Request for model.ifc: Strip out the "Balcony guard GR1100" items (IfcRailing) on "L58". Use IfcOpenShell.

First a look at what the model holds.

```python
import ifcopenshell
import ifcopenshell.util.element

model = ifcopenshell.open("model.ifc")
print(model.schema)
storey = next(s for s in model.by_type("IfcBuildingStorey") if s.Name == "L58")
railings = [e for e in ifcopenshell.util.element.get_decomposition(storey) if e.is_a("IfcRailing")]
seen = {}
for e in railings:
    element_type = ifcopenshell.util.element.get_type(e)
    name = element_type.Name if element_type not in (None, e) else None
    seen[name] = seen.get(name, 0) + 1
for name, count in sorted(seen.items(), key=str):
    print(count, "x", name)
```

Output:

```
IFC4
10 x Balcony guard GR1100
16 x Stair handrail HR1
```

```python
import ifcopenshell
import ifcopenshell.api.root
import ifcopenshell.util.element

model = ifcopenshell.open("model.ifc")

storey = next(s for s in model.by_type("IfcBuildingStorey") if s.Name == "L58")
railings = [e for e in ifcopenshell.util.element.get_decomposition(storey) if e.is_a("IfcRailing")]
targets = [e for e in railings if (t := ifcopenshell.util.element.get_type(e)) not in (None, e) and t.Name == "Balcony guard GR1100"]

for e in targets:
    ifcopenshell.api.root.remove_product(model, product=e)
print(len(targets), "removed")

model.write("model_rev.ifc")
```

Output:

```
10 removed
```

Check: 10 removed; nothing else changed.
